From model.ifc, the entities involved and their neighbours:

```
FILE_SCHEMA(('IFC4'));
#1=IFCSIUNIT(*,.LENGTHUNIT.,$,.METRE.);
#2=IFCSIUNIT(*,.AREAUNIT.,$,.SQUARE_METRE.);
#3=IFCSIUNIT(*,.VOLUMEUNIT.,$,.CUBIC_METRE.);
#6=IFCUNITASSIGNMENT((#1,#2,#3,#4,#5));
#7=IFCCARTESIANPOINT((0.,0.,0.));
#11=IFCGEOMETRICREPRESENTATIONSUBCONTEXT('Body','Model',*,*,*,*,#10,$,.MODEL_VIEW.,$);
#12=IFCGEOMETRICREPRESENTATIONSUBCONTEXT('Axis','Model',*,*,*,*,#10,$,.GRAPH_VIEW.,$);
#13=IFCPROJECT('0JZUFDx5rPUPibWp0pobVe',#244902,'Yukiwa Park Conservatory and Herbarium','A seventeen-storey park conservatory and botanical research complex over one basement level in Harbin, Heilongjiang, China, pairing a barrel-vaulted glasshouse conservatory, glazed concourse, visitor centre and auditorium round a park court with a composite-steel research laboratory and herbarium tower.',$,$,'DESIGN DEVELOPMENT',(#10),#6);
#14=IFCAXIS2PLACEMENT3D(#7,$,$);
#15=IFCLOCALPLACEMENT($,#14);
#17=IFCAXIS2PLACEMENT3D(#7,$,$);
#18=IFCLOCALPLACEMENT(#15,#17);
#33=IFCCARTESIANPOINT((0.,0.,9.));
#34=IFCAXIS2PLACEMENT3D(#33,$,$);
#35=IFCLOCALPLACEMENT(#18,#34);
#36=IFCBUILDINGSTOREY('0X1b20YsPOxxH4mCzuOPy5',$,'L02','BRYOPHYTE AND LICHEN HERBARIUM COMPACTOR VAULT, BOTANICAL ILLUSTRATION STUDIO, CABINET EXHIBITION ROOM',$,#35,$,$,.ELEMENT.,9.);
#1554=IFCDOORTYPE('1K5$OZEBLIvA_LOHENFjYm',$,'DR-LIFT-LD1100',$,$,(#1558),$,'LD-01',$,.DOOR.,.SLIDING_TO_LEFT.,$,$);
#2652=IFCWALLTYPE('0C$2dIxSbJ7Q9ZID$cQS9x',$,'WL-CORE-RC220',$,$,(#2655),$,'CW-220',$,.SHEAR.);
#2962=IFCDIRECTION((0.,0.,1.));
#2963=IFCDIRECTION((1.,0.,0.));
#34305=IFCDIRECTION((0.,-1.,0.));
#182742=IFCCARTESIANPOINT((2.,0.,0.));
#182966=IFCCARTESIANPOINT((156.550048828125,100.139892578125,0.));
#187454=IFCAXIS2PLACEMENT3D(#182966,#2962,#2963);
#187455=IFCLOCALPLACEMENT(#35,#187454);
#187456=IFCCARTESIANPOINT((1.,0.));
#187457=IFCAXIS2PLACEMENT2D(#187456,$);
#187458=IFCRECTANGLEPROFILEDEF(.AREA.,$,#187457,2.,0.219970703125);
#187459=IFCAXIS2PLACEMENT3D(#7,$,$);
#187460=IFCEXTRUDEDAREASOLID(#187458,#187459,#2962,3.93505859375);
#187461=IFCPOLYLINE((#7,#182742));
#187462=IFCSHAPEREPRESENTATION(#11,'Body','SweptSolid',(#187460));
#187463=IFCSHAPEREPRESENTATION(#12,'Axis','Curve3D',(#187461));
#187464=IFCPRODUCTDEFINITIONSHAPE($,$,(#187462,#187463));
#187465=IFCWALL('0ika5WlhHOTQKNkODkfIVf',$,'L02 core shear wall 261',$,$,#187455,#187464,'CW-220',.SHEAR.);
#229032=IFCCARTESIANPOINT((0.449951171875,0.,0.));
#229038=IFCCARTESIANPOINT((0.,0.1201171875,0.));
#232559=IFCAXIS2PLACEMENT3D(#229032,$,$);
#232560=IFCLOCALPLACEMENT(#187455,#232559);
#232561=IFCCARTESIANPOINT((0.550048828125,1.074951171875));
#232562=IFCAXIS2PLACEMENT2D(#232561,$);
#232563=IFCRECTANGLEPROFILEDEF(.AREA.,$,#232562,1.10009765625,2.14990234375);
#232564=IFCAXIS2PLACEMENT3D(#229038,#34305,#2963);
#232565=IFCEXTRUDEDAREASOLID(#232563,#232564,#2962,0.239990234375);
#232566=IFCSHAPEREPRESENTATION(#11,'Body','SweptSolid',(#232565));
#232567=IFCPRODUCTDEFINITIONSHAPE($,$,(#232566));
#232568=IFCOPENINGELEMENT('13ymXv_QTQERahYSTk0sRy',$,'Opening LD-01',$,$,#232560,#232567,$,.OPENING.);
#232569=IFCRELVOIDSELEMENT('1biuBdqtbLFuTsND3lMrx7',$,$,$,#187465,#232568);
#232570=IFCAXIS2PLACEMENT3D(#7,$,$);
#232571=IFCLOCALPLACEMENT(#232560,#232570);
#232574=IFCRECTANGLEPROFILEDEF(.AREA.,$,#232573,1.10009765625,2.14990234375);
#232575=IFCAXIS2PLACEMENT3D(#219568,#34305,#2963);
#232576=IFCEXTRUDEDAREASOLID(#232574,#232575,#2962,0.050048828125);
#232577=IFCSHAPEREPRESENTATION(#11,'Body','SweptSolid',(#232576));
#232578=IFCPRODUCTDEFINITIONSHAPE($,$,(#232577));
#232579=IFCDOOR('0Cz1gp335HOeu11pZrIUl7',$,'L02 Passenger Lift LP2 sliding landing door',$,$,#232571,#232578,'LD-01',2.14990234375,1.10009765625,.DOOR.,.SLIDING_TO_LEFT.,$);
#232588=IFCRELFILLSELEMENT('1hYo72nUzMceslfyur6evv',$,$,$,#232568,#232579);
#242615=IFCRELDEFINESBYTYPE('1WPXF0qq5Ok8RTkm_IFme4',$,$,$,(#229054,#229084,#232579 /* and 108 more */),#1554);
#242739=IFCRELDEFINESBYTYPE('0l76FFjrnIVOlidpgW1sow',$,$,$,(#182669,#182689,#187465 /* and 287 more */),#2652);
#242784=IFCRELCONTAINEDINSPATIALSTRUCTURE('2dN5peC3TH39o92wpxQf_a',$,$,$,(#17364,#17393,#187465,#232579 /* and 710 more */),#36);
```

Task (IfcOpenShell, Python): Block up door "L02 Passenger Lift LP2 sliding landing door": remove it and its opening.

```python
import ifcopenshell
import ifcopenshell.api.feature
import ifcopenshell.api.root
import ifcopenshell.geom
import ifcopenshell.util.shape

model = ifcopenshell.open("model.ifc")
settings = ifcopenshell.geom.settings()


def volume(element):
    """Net volume in cubic metres, openings subtracted."""
    shape = ifcopenshell.geom.create_shape(settings, element)
    return ifcopenshell.util.shape.get_volume(shape.geometry)


door = model.by_guid("0Cz1gp335HOeu11pZrIUl7")
opening = door.FillsVoids[0].RelatingOpeningElement
wall = opening.VoidsElements[0].RelatingBuildingElement
before = volume(wall)

ifcopenshell.api.root.remove_product(model, product=door)
ifcopenshell.api.feature.remove_feature(model, feature=opening)

after = volume(wall)

print(f"wall volume {before:.3f} -> {after:.3f} m3")

model.write("model_v2.ifc")
```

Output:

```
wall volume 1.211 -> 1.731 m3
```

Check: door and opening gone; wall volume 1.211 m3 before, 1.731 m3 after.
